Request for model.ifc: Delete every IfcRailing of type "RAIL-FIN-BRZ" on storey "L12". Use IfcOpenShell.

First a look at what the model holds.

```python
import ifcopenshell
import ifcopenshell.util.element

model = ifcopenshell.open("model.ifc")
print(model.schema)
storey = next(s for s in model.by_type("IfcBuildingStorey") if s.Name == "L12")
railings = [e for e in ifcopenshell.util.element.get_decomposition(storey) if e.is_a("IfcRailing")]
seen = {}
for e in railings:
    element_type = ifcopenshell.util.element.get_type(e)
    name = element_type.Name if element_type not in (None, e) else None
    seen[name] = seen.get(name, 0) + 1
for name, count in sorted(seen.items(), key=str):
    print(count, "x", name)
```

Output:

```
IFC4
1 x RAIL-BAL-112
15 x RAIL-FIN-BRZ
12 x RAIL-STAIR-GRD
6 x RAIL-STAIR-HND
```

```python
import ifcopenshell
import ifcopenshell.api.root
import ifcopenshell.util.element

model = ifcopenshell.open("model.ifc")

storey = next(s for s in model.by_type("IfcBuildingStorey") if s.Name == "L12")
railings = [e for e in ifcopenshell.util.element.get_decomposition(storey) if e.is_a("IfcRailing")]
targets = [e for e in railings if (t := ifcopenshell.util.element.get_type(e)) not in (None, e) and t.Name == "RAIL-FIN-BRZ"]

for e in targets:
    ifcopenshell.api.root.remove_product(model, product=e)
print(len(targets), "removed")

model.write("model_v2.ifc")
```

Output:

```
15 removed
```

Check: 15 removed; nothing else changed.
